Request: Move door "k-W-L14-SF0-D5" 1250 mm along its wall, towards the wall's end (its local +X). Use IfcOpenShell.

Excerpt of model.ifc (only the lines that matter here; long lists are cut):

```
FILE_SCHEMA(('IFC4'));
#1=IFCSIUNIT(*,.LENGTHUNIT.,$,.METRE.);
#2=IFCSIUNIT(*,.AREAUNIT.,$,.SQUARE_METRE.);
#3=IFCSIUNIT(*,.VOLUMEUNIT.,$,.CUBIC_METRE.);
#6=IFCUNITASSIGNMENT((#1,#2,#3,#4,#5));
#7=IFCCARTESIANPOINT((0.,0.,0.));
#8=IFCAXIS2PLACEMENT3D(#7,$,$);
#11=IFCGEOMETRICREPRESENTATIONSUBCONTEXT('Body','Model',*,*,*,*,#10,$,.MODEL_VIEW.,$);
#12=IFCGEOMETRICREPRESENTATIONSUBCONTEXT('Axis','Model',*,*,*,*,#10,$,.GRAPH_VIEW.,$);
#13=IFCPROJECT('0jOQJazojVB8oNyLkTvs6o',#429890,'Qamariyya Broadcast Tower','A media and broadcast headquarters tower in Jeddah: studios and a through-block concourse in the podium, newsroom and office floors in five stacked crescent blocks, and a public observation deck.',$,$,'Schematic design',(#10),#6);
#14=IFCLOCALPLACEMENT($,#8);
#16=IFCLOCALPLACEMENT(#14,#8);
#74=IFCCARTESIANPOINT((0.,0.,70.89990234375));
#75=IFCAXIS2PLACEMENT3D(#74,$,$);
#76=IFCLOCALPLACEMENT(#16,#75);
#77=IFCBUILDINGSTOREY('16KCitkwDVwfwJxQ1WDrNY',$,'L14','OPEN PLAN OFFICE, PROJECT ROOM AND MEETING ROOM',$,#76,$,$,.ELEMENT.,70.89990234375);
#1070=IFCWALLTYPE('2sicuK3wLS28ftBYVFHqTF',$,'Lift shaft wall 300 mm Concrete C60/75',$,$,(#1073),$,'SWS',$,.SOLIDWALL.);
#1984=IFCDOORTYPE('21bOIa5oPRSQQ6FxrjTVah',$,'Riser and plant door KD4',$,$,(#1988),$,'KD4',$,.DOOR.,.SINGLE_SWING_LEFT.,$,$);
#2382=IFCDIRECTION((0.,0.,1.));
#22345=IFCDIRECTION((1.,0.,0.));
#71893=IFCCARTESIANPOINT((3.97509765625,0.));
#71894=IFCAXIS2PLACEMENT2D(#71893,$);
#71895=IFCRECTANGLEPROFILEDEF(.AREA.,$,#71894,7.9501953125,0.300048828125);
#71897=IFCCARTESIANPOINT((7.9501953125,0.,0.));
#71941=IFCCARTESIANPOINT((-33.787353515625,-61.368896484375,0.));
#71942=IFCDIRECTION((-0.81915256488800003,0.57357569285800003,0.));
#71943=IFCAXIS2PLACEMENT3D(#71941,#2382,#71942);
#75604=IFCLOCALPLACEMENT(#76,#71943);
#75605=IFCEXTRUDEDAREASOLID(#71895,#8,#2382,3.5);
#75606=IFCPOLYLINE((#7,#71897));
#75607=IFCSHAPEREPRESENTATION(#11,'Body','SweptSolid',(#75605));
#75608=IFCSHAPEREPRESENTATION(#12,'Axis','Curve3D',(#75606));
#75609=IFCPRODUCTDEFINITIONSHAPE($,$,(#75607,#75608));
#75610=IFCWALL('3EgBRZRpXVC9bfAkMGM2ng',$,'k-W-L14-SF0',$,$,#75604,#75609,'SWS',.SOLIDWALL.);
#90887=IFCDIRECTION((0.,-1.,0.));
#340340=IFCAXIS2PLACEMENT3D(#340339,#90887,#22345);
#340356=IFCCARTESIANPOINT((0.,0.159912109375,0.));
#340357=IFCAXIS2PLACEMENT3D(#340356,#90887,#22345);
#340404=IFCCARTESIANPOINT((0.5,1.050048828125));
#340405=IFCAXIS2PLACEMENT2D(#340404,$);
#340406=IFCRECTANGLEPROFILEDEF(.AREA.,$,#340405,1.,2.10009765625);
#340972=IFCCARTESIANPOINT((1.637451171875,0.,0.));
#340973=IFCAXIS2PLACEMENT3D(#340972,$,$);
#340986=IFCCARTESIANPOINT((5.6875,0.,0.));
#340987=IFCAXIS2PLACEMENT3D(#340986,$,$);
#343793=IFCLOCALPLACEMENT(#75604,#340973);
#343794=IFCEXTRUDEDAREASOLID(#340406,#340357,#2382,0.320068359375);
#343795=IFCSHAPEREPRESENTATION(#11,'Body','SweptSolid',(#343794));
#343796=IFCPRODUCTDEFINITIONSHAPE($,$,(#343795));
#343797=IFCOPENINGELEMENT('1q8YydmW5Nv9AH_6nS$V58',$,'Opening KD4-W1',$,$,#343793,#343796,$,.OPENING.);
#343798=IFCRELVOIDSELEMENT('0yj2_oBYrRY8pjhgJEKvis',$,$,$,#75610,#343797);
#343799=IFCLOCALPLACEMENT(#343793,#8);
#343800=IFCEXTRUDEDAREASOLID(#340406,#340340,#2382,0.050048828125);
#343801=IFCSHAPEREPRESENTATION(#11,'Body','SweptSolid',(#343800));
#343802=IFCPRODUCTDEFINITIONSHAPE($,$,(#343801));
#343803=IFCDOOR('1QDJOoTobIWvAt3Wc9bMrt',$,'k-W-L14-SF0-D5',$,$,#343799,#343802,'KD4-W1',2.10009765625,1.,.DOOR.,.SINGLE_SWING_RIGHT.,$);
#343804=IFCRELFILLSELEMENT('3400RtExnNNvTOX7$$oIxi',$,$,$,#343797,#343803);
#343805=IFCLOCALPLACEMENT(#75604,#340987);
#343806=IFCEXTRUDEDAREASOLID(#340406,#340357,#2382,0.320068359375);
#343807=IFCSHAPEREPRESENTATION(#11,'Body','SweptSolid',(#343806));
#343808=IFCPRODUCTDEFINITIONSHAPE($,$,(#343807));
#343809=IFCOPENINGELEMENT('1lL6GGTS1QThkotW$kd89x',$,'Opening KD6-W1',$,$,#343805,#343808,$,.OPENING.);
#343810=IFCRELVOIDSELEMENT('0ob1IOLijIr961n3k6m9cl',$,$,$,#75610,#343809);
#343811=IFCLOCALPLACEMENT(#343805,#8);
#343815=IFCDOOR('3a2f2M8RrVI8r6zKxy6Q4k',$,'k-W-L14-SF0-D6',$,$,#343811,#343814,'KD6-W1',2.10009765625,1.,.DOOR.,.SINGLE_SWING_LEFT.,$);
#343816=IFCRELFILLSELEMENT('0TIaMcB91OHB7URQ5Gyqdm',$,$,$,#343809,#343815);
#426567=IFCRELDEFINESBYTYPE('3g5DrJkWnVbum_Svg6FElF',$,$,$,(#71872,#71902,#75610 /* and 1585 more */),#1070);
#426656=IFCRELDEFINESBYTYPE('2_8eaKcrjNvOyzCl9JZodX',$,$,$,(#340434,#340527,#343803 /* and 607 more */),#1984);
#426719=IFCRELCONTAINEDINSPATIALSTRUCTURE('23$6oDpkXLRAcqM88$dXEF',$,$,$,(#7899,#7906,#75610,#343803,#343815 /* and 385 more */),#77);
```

```python
import ifcopenshell
import ifcopenshell.api.geometry
import ifcopenshell.util.placement
import ifcopenshell.util.unit

model = ifcopenshell.open("model.ifc")
unit_scale = ifcopenshell.util.unit.calculate_unit_scale(model)

door = model.by_guid("1QDJOoTobIWvAt3Wc9bMrt")
opening = door.FillsVoids[0].RelatingOpeningElement
wall = opening.VoidsElements[0].RelatingBuildingElement

wall_matrix = ifcopenshell.util.placement.get_local_placement(wall.ObjectPlacement)
shift = wall_matrix[:3, 0] * 1.25 / unit_scale
before = ifcopenshell.util.placement.get_local_placement(door.ObjectPlacement)[:3, 3].copy()

# The door is placed relative to its opening, so it follows when the opening moves.
matrix = ifcopenshell.util.placement.get_local_placement(opening.ObjectPlacement)
matrix[:3, 3] += shift
ifcopenshell.api.geometry.edit_object_placement(
    model, product=opening, matrix=matrix, is_si=False, should_transform_children=True
)

after = ifcopenshell.util.placement.get_local_placement(door.ObjectPlacement)[:3, 3]
print("door moved by", (after - before).round(3) + 0.0)

model.write("model_updated.ifc")
```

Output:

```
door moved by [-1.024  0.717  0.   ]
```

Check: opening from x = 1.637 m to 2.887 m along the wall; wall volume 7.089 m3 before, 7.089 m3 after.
